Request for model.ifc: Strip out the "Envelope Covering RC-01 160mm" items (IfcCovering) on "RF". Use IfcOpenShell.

First a look at what the model holds.

```python
import ifcopenshell
import ifcopenshell.util.element

model = ifcopenshell.open("model.ifc")
print(model.schema)
storey = next(s for s in model.by_type("IfcBuildingStorey") if s.Name == "RF")
coverings = [e for e in ifcopenshell.util.element.get_decomposition(storey) if e.is_a("IfcCovering")]
seen = {}
for e in coverings:
    element_type = ifcopenshell.util.element.get_type(e)
    name = element_type.Name if element_type not in (None, e) else None
    seen[name] = seen.get(name, 0) + 1
for name, count in sorted(seen.items(), key=str):
    print(count, "x", name)
```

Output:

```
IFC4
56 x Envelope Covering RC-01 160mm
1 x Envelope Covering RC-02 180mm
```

```python
import ifcopenshell
import ifcopenshell.api.root
import ifcopenshell.util.element

model = ifcopenshell.open("model.ifc")

storey = next(s for s in model.by_type("IfcBuildingStorey") if s.Name == "RF")
coverings = [e for e in ifcopenshell.util.element.get_decomposition(storey) if e.is_a("IfcCovering")]
targets = [e for e in coverings if (t := ifcopenshell.util.element.get_type(e)) not in (None, e) and t.Name == "Envelope Covering RC-01 160mm"]

for e in targets:
    ifcopenshell.api.root.remove_product(model, product=e)
print(len(targets), "removed")

model.write("model_edited.ifc")
```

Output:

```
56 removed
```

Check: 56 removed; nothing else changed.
